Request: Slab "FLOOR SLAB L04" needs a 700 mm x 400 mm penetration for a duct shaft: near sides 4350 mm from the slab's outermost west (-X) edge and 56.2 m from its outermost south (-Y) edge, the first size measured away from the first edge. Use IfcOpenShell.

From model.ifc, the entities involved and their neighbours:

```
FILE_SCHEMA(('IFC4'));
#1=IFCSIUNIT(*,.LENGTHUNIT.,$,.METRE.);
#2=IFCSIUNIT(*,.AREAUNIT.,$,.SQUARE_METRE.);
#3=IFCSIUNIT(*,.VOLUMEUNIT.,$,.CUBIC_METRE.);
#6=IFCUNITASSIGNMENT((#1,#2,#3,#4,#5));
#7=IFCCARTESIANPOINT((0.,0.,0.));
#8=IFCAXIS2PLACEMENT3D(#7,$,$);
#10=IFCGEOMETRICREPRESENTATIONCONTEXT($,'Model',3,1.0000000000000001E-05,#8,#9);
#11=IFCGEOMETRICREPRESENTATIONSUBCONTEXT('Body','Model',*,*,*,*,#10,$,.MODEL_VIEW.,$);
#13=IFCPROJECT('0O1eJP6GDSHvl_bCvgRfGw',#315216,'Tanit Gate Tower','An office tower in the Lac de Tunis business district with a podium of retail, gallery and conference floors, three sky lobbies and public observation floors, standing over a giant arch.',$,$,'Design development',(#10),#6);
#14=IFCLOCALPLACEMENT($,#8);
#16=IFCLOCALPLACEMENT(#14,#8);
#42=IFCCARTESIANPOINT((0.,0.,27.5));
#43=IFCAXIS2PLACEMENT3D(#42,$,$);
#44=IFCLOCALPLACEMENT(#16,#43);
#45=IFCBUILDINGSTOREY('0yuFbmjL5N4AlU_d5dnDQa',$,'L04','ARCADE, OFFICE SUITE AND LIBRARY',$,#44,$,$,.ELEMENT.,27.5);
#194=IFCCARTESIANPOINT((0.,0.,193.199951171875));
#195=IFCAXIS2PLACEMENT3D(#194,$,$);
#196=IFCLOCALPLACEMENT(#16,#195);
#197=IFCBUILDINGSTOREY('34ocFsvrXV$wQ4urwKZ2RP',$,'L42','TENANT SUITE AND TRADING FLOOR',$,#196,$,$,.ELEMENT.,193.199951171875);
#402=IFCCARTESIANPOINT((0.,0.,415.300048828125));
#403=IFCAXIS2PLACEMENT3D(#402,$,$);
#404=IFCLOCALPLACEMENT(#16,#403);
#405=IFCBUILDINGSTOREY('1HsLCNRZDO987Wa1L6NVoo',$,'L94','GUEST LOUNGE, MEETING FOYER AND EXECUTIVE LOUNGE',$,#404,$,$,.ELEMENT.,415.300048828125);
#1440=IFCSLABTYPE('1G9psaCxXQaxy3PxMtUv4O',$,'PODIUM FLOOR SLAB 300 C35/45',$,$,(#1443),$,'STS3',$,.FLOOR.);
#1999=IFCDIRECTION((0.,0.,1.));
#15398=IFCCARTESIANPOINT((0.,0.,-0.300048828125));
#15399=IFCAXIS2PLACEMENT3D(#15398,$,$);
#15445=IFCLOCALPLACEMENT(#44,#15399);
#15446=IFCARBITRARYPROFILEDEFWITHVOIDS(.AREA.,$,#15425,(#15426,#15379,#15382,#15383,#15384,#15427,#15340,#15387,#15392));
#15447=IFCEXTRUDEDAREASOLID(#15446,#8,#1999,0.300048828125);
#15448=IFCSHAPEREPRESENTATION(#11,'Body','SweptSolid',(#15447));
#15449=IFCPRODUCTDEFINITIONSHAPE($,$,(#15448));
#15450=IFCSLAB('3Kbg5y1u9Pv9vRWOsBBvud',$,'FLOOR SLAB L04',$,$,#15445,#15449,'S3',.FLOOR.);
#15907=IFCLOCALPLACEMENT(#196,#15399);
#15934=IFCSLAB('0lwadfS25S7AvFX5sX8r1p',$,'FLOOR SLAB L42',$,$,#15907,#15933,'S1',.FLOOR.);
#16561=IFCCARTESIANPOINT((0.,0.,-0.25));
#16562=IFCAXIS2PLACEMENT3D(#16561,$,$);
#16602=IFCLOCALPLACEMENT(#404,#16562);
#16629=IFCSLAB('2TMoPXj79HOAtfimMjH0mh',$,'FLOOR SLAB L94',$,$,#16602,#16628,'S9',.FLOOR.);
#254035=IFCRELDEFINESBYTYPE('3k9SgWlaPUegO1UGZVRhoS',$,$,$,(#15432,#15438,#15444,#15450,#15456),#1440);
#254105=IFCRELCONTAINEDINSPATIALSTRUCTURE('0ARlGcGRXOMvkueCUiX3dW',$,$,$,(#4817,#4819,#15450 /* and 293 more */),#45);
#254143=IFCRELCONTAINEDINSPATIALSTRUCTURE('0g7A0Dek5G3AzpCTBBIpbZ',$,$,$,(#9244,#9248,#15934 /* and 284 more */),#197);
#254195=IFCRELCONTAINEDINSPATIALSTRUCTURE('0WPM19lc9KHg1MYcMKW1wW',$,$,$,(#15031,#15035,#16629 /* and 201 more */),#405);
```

```python
import numpy as np
import ifcopenshell
import ifcopenshell.api.feature
import ifcopenshell.api.geometry
import ifcopenshell.api.root
import ifcopenshell.geom
import ifcopenshell.util.placement
import ifcopenshell.util.representation
import ifcopenshell.util.shape
import ifcopenshell.util.unit

model = ifcopenshell.open("model.ifc")
unit_scale = ifcopenshell.util.unit.calculate_unit_scale(model)
settings = ifcopenshell.geom.settings()


def volume(element):
    """Net volume in cubic metres, openings subtracted."""
    shape = ifcopenshell.geom.create_shape(settings, element)
    return ifcopenshell.util.shape.get_volume(shape.geometry)


slab = model.by_guid("3Kbg5y1u9Pv9vRWOsBBvud")
before = volume(slab)

# Extent in the slab's own axes, in metres. The edges named are its -X and -Y sides.
slab_shape = ifcopenshell.geom.create_shape(settings, slab)
vertices = ifcopenshell.util.shape.get_vertices(slab_shape.geometry)
x_min, y_min, bottom = vertices.min(axis=0)
top = vertices[:, 2].max()

opening = ifcopenshell.api.root.create_entity(model, ifc_class="IfcOpeningElement", name="Duct shaft opening", predefined_type="OPENING")
context = ifcopenshell.util.representation.get_context(model, "Model", "Body", "MODEL_VIEW")
width, depth = 0.7, 0.4
outline = [(0.0, 0.0), (width, 0.0), (width, depth), (0.0, depth), (0.0, 0.0)]
# Overshoot both faces by 50 mm so the cut is clean.
shape = ifcopenshell.api.geometry.add_slab_representation(
    model, context=context, depth=top - bottom + 0.1, polyline=outline
)
ifcopenshell.api.geometry.assign_representation(model, product=opening, representation=shape)

matrix = ifcopenshell.util.placement.get_local_placement(slab.ObjectPlacement)
matrix[:, 3] = matrix @ np.append(np.array([x_min + 4.35, y_min + 56.2, bottom - 0.05]) / unit_scale, 1.0)
ifcopenshell.api.geometry.edit_object_placement(model, product=opening, matrix=matrix, is_si=False)
ifcopenshell.api.feature.add_feature(model, feature=opening, element=slab)

after = volume(slab)

print(f"slab volume {before:.3f} -> {after:.3f} m3")

model.write("model_updated.ifc")
```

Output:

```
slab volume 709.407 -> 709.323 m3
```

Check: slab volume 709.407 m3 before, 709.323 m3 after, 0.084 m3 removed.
